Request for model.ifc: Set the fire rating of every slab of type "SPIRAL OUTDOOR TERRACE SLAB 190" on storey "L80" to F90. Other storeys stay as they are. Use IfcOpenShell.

First a look at what the model holds.

```python
import ifcopenshell
import ifcopenshell.util.element

model = ifcopenshell.open("model.ifc")
print(model.schema)
storey = next(s for s in model.by_type("IfcBuildingStorey") if s.Name == "L80")
slabs = [e for e in ifcopenshell.util.element.get_decomposition(storey) if e.is_a("IfcSlab")]
seen = {}
for e in slabs:
    element_type = ifcopenshell.util.element.get_type(e)
    key = (element_type.Name if element_type != e and element_type else None, ifcopenshell.util.element.get_pset(e, "Pset_SlabCommon", "FireRating"))
    seen[key] = seen.get(key, 0) + 1
for (name, value), count in sorted(seen.items(), key=str):
    print(count, "x", name, "|", value)
```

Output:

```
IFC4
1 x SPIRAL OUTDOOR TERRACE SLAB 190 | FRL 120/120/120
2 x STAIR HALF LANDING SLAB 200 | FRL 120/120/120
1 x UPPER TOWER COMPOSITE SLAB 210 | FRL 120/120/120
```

```python
import ifcopenshell
import ifcopenshell.api.pset
import ifcopenshell.util.element

model = ifcopenshell.open("model.ifc")

storey = next(s for s in model.by_type("IfcBuildingStorey") if s.Name == "L80")
slabs = [e for e in ifcopenshell.util.element.get_decomposition(storey) if e.is_a("IfcSlab")]

count = 0
for e in slabs:
    element_type = ifcopenshell.util.element.get_type(e)
    if element_type in (None, e) or element_type.Name != "SPIRAL OUTDOOR TERRACE SLAB 190":
        continue
    # add_pset returns the element's existing set when there is one.
    pset = ifcopenshell.api.pset.add_pset(model, product=e, name="Pset_SlabCommon")
    ifcopenshell.api.pset.edit_pset(model, pset=pset, properties={"FireRating": "F90"})
    count += 1

print(count, "slabs updated")

model.write("model_updated.ifc")
```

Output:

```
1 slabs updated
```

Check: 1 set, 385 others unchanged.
